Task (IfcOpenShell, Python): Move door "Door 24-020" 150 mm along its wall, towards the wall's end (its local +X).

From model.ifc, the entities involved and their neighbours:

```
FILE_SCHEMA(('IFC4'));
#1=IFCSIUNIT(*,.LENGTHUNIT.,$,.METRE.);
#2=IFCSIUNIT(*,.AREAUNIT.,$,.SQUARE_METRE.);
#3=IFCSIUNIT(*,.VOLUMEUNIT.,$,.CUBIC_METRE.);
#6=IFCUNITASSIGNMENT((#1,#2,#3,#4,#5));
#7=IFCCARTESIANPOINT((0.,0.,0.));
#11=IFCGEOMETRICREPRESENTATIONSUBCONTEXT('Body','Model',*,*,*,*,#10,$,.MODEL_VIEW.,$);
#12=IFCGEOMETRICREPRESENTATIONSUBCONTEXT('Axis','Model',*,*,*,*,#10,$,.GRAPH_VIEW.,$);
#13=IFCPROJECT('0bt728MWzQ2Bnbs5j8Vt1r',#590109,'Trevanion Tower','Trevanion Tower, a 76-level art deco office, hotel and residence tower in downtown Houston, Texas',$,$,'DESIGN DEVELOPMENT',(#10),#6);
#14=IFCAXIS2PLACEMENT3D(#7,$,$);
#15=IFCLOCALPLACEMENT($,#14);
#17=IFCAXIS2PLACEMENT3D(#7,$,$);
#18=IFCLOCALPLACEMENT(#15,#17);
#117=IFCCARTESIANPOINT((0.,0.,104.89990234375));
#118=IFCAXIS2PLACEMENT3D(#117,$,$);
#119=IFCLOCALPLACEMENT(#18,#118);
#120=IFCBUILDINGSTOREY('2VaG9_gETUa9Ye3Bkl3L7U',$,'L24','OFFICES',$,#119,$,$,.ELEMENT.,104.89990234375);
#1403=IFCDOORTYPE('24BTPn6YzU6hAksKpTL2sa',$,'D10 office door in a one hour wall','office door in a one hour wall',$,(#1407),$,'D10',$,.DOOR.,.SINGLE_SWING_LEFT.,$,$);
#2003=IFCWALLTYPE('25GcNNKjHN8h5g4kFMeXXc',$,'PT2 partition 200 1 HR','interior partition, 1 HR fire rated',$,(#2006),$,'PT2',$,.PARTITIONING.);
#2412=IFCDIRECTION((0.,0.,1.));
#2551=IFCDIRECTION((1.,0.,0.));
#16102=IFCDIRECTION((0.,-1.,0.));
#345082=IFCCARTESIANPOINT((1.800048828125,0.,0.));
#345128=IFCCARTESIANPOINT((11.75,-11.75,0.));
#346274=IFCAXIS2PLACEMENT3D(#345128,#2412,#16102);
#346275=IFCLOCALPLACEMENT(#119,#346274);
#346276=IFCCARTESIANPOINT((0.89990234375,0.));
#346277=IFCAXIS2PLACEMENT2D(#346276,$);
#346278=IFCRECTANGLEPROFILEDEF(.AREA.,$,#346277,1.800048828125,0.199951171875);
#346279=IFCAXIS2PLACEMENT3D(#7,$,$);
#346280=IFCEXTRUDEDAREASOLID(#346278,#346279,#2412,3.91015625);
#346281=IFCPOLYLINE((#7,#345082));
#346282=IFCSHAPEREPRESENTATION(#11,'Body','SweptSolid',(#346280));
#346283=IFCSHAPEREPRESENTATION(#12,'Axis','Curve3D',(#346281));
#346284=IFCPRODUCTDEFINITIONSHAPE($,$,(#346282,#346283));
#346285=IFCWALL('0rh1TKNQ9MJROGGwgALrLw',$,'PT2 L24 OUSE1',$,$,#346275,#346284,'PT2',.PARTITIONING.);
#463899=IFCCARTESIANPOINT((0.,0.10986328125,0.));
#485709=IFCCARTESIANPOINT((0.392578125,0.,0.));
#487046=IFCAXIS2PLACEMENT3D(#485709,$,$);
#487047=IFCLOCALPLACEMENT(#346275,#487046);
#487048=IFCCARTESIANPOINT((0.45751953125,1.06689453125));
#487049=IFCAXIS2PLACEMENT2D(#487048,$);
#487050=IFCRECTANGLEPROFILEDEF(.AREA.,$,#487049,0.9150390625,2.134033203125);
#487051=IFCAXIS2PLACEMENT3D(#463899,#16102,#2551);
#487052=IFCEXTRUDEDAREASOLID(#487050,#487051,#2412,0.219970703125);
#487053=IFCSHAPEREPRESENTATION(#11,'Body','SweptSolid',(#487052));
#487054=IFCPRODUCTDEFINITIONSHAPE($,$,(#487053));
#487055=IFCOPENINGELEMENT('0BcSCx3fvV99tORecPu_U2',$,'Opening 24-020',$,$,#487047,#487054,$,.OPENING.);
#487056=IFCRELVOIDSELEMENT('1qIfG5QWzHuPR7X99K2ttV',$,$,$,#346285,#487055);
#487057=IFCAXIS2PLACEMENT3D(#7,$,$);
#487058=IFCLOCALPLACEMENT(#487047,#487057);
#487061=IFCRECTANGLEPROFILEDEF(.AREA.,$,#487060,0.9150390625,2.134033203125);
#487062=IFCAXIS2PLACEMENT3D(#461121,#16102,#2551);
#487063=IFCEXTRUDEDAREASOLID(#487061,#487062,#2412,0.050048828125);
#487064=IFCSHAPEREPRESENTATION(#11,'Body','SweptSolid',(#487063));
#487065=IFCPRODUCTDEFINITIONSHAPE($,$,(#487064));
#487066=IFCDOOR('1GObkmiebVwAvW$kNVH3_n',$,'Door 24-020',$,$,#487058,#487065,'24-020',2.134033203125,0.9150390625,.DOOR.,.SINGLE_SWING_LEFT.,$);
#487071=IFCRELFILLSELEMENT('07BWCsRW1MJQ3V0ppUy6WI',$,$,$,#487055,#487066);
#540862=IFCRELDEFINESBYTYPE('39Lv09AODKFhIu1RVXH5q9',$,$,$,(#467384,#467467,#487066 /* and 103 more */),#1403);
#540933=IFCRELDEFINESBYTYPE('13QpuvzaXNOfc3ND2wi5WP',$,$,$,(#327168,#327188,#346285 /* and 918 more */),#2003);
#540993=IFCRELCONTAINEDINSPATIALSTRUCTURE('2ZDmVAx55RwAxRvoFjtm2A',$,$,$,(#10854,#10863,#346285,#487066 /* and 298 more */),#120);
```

```python
import ifcopenshell
import ifcopenshell.api.geometry
import ifcopenshell.util.placement

model = ifcopenshell.open("model.ifc")

door = model.by_guid("1GObkmiebVwAvW$kNVH3_n")
opening = door.FillsVoids[0].RelatingOpeningElement
wall = opening.VoidsElements[0].RelatingBuildingElement

wall_matrix = ifcopenshell.util.placement.get_local_placement(wall.ObjectPlacement)
shift = wall_matrix[:3, 0] * 0.15
before = ifcopenshell.util.placement.get_local_placement(door.ObjectPlacement)[:3, 3].copy()

# The door is placed relative to its opening, so it follows when the opening moves.
matrix = ifcopenshell.util.placement.get_local_placement(opening.ObjectPlacement)
matrix[:3, 3] += shift
ifcopenshell.api.geometry.edit_object_placement(
    model, product=opening, matrix=matrix, is_si=False, should_transform_children=True
)

after = ifcopenshell.util.placement.get_local_placement(door.ObjectPlacement)[:3, 3]
print("door moved by", (after - before).round(3) + 0.0)

model.write("model_rev.ifc")
```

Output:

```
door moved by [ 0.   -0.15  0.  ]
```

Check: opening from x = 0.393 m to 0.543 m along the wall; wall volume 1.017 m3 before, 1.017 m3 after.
